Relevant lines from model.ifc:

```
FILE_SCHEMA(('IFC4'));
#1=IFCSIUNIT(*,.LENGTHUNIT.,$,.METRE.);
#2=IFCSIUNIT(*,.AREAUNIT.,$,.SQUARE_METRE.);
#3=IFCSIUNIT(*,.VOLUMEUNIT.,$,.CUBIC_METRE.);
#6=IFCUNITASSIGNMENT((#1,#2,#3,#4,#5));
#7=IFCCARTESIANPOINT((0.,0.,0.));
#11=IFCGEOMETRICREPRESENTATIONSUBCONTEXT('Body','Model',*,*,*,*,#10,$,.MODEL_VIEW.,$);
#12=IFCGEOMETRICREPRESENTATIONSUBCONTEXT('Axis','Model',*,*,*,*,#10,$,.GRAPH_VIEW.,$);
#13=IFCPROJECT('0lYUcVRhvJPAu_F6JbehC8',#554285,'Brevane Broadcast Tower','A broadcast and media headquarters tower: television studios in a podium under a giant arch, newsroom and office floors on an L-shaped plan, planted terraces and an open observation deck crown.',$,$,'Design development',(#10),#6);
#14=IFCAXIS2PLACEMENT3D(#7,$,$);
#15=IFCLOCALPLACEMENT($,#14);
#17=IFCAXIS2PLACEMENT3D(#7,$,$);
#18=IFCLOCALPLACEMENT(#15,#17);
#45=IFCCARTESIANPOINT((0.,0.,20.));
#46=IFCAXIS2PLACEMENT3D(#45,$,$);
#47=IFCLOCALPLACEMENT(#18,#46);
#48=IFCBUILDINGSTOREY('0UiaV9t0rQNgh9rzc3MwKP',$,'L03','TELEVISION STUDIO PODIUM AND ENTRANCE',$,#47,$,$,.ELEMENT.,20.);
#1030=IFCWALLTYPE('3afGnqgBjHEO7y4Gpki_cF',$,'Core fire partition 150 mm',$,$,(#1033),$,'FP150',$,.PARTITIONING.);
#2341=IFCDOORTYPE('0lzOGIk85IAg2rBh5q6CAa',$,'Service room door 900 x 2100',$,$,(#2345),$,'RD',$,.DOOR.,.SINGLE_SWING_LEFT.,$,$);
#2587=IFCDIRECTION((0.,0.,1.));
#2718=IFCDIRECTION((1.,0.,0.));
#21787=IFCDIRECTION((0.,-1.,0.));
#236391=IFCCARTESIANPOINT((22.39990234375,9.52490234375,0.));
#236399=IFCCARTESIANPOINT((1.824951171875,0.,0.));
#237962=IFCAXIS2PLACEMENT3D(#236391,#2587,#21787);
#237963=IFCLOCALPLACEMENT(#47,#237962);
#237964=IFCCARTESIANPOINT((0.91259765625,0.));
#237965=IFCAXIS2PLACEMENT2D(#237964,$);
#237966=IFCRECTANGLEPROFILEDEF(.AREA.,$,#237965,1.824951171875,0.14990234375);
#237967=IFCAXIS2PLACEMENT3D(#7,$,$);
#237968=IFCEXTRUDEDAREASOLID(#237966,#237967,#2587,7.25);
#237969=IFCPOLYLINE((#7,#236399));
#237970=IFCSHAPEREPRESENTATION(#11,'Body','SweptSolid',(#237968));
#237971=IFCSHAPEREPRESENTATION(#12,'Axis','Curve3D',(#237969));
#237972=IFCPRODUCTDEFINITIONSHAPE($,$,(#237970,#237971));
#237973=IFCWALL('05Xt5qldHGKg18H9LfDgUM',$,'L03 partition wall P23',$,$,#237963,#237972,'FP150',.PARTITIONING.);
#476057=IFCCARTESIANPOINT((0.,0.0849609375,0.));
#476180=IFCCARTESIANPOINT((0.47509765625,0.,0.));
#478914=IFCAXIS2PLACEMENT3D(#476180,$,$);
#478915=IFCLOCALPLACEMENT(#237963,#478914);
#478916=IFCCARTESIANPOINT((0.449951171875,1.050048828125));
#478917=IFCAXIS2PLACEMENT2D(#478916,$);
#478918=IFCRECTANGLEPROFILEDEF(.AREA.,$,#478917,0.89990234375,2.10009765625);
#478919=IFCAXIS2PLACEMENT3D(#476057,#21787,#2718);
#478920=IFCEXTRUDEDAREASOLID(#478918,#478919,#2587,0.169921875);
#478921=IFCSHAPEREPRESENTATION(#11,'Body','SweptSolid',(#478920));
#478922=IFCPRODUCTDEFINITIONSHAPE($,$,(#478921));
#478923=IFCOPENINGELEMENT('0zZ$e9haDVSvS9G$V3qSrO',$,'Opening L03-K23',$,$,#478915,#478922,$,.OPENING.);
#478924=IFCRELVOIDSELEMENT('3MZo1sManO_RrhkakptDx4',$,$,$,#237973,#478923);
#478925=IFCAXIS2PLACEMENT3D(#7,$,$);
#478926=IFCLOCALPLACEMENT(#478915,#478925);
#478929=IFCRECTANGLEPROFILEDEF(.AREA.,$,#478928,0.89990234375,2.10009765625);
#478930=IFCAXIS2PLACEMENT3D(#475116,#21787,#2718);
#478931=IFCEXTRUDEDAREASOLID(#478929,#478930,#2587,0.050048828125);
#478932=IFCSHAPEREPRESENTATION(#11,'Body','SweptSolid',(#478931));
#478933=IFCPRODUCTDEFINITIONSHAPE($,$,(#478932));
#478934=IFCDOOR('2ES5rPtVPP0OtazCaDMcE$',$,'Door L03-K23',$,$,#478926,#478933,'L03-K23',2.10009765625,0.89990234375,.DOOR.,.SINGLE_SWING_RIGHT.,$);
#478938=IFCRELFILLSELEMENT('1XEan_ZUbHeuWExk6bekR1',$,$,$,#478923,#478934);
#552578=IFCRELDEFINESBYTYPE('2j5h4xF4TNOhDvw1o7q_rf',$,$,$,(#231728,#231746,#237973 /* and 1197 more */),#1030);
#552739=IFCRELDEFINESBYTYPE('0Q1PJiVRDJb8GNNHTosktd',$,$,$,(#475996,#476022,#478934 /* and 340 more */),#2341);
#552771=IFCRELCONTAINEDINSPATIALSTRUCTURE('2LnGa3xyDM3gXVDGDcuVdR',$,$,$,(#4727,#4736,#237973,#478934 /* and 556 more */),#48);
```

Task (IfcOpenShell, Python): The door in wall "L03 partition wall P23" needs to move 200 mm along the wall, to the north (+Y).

```python
import ifcopenshell
import ifcopenshell.api.geometry
import ifcopenshell.util.placement
import ifcopenshell.util.unit

model = ifcopenshell.open("model.ifc")
unit_scale = ifcopenshell.util.unit.calculate_unit_scale(model)

door = model.by_guid("2ES5rPtVPP0OtazCaDMcE$")
opening = door.FillsVoids[0].RelatingOpeningElement
wall = opening.VoidsElements[0].RelatingBuildingElement

wall_matrix = ifcopenshell.util.placement.get_local_placement(wall.ObjectPlacement)
shift = wall_matrix[:3, 0] * -0.2 / unit_scale
before = ifcopenshell.util.placement.get_local_placement(door.ObjectPlacement)[:3, 3].copy()

# The door is placed relative to its opening, so it follows when the opening moves.
matrix = ifcopenshell.util.placement.get_local_placement(opening.ObjectPlacement)
matrix[:3, 3] += shift
ifcopenshell.api.geometry.edit_object_placement(
    model, product=opening, matrix=matrix, is_si=False, should_transform_children=True
)

after = ifcopenshell.util.placement.get_local_placement(door.ObjectPlacement)[:3, 3]
print("door moved by", (after - before).round(3) + 0.0)

model.write("model-out.ifc")
```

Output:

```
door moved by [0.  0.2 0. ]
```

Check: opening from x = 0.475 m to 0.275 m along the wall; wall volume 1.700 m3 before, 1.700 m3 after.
